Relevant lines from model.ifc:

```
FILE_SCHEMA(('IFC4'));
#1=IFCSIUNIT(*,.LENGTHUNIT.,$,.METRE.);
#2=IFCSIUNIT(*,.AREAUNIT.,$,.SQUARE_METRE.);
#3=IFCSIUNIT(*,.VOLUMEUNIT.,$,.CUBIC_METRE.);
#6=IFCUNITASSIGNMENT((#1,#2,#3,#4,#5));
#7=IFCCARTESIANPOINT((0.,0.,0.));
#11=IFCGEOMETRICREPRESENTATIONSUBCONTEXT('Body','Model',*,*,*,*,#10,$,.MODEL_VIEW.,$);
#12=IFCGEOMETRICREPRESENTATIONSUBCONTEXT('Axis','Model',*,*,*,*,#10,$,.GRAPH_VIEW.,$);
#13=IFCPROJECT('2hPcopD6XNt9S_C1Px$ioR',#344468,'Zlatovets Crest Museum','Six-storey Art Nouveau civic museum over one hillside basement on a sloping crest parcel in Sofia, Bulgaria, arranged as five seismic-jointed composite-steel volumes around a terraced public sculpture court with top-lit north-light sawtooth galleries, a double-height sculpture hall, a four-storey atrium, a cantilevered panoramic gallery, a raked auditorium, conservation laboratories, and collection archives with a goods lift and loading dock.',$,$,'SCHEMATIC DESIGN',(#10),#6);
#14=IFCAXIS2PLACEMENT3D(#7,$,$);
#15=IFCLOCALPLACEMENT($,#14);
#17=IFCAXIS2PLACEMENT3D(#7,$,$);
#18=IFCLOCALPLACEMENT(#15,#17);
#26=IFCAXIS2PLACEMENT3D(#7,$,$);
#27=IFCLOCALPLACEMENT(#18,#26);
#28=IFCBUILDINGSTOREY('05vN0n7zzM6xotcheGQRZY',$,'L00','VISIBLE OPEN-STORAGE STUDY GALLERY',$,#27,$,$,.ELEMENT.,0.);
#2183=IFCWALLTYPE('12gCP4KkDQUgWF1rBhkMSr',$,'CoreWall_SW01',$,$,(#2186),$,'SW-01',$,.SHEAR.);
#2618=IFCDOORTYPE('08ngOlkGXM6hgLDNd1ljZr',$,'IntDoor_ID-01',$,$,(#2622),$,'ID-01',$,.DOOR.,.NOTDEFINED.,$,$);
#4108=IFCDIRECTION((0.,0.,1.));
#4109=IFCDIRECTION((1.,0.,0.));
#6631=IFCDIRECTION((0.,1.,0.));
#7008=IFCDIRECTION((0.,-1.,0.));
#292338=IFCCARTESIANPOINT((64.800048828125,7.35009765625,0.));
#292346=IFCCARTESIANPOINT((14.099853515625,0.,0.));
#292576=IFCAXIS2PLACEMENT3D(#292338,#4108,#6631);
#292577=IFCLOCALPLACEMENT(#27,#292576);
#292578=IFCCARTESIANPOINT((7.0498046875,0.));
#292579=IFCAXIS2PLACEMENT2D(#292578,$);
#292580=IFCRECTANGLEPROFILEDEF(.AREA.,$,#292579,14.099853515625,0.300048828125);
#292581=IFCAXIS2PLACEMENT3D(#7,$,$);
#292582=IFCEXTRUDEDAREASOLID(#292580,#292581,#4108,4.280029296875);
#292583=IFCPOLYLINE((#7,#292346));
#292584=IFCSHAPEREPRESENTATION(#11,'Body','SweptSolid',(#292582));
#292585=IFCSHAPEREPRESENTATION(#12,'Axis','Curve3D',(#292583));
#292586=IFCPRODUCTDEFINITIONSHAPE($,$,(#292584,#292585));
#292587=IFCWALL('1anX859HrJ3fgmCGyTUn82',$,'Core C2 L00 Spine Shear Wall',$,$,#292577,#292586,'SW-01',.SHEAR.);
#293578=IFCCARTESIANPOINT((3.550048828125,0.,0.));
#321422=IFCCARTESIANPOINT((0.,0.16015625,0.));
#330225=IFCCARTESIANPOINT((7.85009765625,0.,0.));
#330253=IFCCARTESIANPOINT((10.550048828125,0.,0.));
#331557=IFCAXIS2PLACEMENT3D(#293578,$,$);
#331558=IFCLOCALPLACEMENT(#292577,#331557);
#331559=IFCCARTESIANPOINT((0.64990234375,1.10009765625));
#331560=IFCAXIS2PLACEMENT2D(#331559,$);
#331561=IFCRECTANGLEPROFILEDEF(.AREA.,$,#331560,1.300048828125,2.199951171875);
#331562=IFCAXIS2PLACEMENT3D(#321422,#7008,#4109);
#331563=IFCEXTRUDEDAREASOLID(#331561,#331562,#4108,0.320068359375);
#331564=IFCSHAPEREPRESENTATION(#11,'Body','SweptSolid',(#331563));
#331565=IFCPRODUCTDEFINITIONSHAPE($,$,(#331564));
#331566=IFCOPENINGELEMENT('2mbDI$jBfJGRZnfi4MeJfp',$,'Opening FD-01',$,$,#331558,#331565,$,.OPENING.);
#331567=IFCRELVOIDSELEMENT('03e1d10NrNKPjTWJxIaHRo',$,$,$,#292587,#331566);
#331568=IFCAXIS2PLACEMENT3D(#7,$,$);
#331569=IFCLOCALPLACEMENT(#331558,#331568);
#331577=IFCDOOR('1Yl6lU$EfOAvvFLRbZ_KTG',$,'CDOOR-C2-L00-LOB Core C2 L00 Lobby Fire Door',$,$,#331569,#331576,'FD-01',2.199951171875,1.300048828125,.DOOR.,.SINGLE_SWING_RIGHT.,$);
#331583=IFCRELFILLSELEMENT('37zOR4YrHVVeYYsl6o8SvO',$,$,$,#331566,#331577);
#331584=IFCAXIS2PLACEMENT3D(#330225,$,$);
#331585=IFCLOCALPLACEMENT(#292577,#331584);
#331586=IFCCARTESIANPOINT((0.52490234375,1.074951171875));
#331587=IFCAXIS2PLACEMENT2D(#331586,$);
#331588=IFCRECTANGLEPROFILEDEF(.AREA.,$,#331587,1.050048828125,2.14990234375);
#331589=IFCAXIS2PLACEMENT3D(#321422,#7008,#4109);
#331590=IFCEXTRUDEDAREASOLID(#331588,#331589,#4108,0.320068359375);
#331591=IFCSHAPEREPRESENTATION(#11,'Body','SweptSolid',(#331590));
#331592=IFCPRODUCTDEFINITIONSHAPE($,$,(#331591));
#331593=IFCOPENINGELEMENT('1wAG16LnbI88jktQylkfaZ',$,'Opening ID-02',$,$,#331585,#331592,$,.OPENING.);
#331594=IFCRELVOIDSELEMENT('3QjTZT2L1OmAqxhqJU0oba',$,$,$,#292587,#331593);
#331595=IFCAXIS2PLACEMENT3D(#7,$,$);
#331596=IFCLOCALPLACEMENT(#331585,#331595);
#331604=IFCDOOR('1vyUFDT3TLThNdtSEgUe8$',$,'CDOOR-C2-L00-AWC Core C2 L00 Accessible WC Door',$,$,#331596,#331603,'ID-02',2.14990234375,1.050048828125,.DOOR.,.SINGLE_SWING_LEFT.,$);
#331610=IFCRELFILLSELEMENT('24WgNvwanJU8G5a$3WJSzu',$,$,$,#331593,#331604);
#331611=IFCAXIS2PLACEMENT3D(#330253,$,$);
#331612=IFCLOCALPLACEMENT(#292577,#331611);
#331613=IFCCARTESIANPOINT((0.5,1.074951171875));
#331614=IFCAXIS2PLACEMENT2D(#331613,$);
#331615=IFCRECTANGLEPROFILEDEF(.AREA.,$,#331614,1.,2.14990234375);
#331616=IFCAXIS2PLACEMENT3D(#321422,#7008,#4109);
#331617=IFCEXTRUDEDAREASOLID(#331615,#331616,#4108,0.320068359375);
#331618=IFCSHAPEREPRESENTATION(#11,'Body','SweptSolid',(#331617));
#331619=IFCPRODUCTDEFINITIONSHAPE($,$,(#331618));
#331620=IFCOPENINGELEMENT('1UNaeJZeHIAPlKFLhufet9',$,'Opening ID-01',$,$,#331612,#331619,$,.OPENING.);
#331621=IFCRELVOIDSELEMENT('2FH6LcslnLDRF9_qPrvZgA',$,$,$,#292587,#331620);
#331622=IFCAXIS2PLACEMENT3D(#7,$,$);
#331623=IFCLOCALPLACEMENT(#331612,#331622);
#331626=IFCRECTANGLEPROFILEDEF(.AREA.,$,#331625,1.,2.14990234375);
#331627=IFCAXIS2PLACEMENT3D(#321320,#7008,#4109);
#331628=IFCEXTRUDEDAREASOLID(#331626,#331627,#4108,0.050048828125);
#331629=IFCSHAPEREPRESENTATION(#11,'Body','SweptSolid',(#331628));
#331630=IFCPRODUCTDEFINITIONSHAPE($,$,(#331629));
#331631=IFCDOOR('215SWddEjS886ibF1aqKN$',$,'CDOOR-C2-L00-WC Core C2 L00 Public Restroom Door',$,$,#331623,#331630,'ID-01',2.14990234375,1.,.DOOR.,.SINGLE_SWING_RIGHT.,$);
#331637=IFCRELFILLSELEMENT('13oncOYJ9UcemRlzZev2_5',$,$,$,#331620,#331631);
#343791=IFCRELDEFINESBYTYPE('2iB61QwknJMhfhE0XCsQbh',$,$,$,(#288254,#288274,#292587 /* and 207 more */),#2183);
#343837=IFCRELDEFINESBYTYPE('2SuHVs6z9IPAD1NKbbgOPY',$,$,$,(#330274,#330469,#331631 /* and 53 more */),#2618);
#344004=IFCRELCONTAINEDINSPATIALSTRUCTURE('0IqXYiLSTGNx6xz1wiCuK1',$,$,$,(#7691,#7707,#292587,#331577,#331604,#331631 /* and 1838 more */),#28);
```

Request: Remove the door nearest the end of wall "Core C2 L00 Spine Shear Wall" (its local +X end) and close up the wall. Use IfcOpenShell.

```python
import ifcopenshell
import ifcopenshell.api.feature
import ifcopenshell.api.root
import ifcopenshell.geom
import ifcopenshell.util.shape

model = ifcopenshell.open("model.ifc")
settings = ifcopenshell.geom.settings()


def volume(element):
    """Net volume in cubic metres, openings subtracted."""
    shape = ifcopenshell.geom.create_shape(settings, element)
    return ifcopenshell.util.shape.get_volume(shape.geometry)


door = model.by_id(331631)
opening = door.FillsVoids[0].RelatingOpeningElement
wall = opening.VoidsElements[0].RelatingBuildingElement
before = volume(wall)

ifcopenshell.api.root.remove_product(model, product=door)
ifcopenshell.api.feature.remove_feature(model, feature=opening)

after = volume(wall)

print(f"wall volume {before:.3f} -> {after:.3f} m3")

model.write("model_updated.ifc")
```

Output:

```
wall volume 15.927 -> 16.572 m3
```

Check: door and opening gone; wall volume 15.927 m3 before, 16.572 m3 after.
